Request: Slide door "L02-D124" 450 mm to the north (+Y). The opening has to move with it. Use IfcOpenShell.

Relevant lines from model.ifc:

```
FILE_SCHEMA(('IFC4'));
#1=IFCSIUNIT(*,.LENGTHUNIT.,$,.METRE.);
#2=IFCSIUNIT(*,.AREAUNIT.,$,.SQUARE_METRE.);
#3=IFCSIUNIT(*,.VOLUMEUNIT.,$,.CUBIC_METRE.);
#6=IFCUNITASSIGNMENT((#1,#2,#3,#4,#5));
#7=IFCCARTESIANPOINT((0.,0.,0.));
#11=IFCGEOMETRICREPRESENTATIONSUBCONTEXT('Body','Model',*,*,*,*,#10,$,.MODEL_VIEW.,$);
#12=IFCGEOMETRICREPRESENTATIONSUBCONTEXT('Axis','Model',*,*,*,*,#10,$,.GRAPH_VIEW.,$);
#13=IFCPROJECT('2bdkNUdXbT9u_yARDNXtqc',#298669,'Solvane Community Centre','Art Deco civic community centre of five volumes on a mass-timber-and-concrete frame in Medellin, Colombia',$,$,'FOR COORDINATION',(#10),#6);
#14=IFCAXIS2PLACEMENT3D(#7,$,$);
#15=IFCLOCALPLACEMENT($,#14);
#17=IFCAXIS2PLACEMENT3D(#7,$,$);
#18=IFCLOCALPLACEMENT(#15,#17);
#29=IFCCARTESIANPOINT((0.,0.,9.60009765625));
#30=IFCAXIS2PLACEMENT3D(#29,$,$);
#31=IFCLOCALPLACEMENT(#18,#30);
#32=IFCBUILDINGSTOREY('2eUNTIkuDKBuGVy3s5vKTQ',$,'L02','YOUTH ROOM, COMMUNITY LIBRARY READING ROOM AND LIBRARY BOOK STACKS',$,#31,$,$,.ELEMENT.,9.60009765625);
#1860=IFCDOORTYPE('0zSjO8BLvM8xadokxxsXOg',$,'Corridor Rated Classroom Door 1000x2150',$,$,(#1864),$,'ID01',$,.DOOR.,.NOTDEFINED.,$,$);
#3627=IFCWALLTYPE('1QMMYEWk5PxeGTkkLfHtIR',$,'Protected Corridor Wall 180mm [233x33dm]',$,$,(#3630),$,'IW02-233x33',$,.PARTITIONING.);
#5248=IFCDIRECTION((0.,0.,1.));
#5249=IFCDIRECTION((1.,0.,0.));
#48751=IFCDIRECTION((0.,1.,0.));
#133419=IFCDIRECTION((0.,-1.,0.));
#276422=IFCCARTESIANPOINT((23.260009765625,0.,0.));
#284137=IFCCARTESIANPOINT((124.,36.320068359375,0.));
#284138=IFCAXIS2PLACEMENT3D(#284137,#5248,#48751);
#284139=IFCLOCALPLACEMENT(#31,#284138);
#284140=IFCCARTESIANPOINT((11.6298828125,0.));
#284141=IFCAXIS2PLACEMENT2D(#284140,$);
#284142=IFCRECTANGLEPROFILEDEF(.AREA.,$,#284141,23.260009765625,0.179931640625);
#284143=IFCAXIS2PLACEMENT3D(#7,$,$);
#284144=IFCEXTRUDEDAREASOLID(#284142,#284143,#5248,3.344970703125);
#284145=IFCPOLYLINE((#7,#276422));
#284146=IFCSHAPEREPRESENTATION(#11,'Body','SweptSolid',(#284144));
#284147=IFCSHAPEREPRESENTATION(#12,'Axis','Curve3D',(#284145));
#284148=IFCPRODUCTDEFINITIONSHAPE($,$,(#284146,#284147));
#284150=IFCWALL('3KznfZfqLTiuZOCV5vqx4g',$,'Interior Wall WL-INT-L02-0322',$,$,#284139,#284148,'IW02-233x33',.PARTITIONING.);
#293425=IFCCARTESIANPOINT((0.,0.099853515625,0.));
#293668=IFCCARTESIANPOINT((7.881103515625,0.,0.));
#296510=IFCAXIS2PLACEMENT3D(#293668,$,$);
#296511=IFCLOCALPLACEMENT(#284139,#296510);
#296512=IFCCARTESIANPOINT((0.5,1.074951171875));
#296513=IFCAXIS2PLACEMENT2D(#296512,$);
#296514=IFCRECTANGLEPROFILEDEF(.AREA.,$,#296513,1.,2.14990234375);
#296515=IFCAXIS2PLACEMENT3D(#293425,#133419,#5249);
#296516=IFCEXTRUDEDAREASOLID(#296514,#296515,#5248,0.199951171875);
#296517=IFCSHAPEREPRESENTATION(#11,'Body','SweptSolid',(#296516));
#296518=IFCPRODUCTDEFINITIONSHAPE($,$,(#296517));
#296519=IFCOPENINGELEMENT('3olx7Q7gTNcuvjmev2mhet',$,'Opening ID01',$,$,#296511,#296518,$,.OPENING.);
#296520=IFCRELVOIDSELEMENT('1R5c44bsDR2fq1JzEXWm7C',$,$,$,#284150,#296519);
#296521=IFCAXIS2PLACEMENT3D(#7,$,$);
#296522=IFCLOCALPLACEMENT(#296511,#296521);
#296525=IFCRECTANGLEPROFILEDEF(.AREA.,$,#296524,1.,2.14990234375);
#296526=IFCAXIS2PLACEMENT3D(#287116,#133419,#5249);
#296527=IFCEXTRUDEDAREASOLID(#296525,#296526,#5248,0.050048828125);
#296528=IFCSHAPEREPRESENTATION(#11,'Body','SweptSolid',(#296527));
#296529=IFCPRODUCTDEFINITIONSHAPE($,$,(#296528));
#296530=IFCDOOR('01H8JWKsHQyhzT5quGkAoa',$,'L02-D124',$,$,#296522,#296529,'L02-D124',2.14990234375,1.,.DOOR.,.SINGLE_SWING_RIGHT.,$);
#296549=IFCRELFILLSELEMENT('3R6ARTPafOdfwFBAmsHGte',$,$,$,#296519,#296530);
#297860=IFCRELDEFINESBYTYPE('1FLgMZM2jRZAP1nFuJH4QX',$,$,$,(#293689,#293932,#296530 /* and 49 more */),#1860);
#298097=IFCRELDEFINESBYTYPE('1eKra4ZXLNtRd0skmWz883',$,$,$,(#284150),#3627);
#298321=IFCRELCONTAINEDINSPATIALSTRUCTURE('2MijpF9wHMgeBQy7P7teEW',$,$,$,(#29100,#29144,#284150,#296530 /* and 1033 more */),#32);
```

```python
import ifcopenshell
import ifcopenshell.api.geometry
import ifcopenshell.util.placement
import ifcopenshell.util.unit

model = ifcopenshell.open("model.ifc")
unit_scale = ifcopenshell.util.unit.calculate_unit_scale(model)

door = model.by_guid("01H8JWKsHQyhzT5quGkAoa")
opening = door.FillsVoids[0].RelatingOpeningElement
wall = opening.VoidsElements[0].RelatingBuildingElement

wall_matrix = ifcopenshell.util.placement.get_local_placement(wall.ObjectPlacement)
shift = wall_matrix[:3, 0] * 0.45 / unit_scale
before = ifcopenshell.util.placement.get_local_placement(door.ObjectPlacement)[:3, 3].copy()

# The door is placed relative to its opening, so it follows when the opening moves.
matrix = ifcopenshell.util.placement.get_local_placement(opening.ObjectPlacement)
matrix[:3, 3] += shift
ifcopenshell.api.geometry.edit_object_placement(
    model, product=opening, matrix=matrix, is_si=False, should_transform_children=True
)

after = ifcopenshell.util.placement.get_local_placement(door.ObjectPlacement)[:3, 3]
print("door moved by", (after - before).round(3) + 0.0)

model.write("model-out.ifc")
```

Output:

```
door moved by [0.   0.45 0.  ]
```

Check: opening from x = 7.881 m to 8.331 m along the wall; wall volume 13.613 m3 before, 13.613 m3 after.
